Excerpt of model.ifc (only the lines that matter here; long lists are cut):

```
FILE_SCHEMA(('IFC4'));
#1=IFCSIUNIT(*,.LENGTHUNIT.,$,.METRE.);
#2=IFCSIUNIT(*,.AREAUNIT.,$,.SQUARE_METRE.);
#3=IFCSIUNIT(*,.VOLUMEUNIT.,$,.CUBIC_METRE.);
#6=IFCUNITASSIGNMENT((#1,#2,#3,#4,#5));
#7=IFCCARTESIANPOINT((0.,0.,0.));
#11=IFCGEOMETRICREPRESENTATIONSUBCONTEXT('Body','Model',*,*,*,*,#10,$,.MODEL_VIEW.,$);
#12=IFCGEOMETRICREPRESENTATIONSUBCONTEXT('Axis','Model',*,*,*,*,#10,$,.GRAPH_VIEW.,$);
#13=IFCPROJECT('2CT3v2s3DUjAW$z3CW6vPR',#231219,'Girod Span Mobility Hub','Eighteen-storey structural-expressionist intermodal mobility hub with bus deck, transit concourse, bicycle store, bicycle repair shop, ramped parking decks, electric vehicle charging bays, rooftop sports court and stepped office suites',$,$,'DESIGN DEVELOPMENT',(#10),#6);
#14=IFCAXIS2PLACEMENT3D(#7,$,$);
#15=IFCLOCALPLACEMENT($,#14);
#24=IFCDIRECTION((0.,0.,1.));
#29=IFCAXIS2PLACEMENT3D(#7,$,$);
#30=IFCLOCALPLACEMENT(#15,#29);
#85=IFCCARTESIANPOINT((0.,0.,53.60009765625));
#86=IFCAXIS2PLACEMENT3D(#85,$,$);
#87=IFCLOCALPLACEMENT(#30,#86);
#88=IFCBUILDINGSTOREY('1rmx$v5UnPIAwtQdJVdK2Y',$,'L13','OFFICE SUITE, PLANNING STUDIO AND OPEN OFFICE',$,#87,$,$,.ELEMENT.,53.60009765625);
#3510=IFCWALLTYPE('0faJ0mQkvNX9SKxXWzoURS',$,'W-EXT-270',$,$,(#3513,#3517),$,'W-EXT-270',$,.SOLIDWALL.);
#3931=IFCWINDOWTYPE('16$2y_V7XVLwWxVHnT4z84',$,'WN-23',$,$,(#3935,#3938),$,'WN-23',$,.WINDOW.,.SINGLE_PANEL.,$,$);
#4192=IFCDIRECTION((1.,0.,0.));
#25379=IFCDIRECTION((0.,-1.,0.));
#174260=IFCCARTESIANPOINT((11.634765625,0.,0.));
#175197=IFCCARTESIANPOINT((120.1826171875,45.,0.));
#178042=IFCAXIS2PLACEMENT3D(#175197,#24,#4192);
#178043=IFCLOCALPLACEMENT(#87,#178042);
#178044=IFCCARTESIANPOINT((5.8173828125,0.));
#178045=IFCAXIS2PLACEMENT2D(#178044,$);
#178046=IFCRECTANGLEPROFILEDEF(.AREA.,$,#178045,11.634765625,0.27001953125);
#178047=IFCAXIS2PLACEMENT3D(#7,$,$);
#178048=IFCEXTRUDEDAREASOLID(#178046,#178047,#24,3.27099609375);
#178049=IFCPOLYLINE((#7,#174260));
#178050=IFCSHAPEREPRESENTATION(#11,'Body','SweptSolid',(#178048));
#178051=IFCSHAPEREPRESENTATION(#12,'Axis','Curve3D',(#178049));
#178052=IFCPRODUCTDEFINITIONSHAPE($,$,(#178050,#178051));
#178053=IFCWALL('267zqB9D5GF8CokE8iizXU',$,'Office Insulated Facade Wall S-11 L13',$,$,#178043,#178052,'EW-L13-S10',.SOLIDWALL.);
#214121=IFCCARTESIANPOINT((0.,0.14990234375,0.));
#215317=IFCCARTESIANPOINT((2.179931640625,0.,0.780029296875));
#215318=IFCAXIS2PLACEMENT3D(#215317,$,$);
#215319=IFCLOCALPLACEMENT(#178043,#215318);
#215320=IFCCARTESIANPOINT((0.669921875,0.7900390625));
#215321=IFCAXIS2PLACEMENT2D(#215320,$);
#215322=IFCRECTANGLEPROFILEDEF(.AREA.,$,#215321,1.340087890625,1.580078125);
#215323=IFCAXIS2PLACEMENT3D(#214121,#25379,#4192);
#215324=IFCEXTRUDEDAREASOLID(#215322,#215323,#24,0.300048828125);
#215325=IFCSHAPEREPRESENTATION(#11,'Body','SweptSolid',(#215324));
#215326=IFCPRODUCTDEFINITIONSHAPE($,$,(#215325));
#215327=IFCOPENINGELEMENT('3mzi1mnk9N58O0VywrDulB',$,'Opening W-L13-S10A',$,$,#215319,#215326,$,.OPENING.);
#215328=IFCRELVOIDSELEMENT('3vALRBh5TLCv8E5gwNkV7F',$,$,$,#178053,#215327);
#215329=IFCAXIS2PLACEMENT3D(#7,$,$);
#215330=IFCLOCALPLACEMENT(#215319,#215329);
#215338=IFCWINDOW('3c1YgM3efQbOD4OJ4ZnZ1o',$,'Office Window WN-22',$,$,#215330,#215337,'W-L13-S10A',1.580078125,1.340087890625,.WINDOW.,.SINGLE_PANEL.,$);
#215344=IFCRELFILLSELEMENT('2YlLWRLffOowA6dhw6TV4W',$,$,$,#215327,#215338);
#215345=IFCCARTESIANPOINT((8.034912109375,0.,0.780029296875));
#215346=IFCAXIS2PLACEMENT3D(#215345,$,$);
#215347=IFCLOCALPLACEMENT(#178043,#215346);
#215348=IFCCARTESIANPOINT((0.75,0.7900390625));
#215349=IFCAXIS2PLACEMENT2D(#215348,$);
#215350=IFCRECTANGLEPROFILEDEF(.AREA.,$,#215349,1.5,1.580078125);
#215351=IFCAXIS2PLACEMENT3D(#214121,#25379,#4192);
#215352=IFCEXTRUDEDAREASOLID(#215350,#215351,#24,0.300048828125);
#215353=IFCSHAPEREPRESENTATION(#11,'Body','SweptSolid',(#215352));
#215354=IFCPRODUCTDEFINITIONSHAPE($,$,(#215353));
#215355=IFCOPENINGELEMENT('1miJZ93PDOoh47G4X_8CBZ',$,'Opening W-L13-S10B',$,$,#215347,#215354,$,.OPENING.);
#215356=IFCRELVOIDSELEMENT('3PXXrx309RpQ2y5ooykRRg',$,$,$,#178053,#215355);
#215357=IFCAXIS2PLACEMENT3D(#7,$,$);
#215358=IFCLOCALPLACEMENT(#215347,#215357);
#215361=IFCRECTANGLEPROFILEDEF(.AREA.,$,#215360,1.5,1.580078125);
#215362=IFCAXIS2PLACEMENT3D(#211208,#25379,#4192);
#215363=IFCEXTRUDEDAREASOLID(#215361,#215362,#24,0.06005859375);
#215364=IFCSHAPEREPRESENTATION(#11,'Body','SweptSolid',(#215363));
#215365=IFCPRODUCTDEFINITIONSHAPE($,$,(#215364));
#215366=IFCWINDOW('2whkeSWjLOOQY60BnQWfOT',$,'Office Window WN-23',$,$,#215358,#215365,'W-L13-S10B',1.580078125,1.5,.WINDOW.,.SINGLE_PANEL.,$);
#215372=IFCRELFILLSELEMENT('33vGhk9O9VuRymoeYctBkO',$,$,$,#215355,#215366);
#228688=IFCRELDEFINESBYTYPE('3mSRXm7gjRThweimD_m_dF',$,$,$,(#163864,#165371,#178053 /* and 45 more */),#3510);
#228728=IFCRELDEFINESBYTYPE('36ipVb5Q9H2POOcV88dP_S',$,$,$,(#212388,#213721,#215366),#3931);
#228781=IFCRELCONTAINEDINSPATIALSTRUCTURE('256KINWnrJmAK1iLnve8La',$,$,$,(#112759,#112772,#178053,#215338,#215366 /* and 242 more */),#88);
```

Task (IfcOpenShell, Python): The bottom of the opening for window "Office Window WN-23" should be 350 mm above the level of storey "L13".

```python
import numpy as np
import ifcopenshell
import ifcopenshell.api.geometry
import ifcopenshell.geom
import ifcopenshell.util.element
import ifcopenshell.util.placement
import ifcopenshell.util.shape
import ifcopenshell.util.unit

model = ifcopenshell.open("model.ifc")
unit_scale = ifcopenshell.util.unit.calculate_unit_scale(model)

window = model.by_guid("2whkeSWjLOOQY60BnQWfOT")
opening = window.FillsVoids[0].RelatingOpeningElement
storey = ifcopenshell.util.element.get_container(window, ifc_class="IfcBuildingStorey")
level = ifcopenshell.util.placement.get_local_placement(storey.ObjectPlacement)[2, 3]

# The opening's origin need not be at the sill, so measure its lowest point.
shape = ifcopenshell.geom.create_shape(ifcopenshell.geom.settings(), opening)
bottom = ifcopenshell.util.shape.get_shape_bottom_elevation(shape, shape.geometry) / unit_scale
dz = level + 0.35 / unit_scale - bottom

shift = np.array([0.0, 0.0, dz])
# The window is placed relative to its opening, so it follows when the opening moves.
matrix = ifcopenshell.util.placement.get_local_placement(opening.ObjectPlacement)
matrix[:3, 3] += shift
ifcopenshell.api.geometry.edit_object_placement(
    model, product=opening, matrix=matrix, is_si=False, should_transform_children=True
)

print(f"moved by {dz * unit_scale:+.3f} m")

model.write("model_v2.ifc")
```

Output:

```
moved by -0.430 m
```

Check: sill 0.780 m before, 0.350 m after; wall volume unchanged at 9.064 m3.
